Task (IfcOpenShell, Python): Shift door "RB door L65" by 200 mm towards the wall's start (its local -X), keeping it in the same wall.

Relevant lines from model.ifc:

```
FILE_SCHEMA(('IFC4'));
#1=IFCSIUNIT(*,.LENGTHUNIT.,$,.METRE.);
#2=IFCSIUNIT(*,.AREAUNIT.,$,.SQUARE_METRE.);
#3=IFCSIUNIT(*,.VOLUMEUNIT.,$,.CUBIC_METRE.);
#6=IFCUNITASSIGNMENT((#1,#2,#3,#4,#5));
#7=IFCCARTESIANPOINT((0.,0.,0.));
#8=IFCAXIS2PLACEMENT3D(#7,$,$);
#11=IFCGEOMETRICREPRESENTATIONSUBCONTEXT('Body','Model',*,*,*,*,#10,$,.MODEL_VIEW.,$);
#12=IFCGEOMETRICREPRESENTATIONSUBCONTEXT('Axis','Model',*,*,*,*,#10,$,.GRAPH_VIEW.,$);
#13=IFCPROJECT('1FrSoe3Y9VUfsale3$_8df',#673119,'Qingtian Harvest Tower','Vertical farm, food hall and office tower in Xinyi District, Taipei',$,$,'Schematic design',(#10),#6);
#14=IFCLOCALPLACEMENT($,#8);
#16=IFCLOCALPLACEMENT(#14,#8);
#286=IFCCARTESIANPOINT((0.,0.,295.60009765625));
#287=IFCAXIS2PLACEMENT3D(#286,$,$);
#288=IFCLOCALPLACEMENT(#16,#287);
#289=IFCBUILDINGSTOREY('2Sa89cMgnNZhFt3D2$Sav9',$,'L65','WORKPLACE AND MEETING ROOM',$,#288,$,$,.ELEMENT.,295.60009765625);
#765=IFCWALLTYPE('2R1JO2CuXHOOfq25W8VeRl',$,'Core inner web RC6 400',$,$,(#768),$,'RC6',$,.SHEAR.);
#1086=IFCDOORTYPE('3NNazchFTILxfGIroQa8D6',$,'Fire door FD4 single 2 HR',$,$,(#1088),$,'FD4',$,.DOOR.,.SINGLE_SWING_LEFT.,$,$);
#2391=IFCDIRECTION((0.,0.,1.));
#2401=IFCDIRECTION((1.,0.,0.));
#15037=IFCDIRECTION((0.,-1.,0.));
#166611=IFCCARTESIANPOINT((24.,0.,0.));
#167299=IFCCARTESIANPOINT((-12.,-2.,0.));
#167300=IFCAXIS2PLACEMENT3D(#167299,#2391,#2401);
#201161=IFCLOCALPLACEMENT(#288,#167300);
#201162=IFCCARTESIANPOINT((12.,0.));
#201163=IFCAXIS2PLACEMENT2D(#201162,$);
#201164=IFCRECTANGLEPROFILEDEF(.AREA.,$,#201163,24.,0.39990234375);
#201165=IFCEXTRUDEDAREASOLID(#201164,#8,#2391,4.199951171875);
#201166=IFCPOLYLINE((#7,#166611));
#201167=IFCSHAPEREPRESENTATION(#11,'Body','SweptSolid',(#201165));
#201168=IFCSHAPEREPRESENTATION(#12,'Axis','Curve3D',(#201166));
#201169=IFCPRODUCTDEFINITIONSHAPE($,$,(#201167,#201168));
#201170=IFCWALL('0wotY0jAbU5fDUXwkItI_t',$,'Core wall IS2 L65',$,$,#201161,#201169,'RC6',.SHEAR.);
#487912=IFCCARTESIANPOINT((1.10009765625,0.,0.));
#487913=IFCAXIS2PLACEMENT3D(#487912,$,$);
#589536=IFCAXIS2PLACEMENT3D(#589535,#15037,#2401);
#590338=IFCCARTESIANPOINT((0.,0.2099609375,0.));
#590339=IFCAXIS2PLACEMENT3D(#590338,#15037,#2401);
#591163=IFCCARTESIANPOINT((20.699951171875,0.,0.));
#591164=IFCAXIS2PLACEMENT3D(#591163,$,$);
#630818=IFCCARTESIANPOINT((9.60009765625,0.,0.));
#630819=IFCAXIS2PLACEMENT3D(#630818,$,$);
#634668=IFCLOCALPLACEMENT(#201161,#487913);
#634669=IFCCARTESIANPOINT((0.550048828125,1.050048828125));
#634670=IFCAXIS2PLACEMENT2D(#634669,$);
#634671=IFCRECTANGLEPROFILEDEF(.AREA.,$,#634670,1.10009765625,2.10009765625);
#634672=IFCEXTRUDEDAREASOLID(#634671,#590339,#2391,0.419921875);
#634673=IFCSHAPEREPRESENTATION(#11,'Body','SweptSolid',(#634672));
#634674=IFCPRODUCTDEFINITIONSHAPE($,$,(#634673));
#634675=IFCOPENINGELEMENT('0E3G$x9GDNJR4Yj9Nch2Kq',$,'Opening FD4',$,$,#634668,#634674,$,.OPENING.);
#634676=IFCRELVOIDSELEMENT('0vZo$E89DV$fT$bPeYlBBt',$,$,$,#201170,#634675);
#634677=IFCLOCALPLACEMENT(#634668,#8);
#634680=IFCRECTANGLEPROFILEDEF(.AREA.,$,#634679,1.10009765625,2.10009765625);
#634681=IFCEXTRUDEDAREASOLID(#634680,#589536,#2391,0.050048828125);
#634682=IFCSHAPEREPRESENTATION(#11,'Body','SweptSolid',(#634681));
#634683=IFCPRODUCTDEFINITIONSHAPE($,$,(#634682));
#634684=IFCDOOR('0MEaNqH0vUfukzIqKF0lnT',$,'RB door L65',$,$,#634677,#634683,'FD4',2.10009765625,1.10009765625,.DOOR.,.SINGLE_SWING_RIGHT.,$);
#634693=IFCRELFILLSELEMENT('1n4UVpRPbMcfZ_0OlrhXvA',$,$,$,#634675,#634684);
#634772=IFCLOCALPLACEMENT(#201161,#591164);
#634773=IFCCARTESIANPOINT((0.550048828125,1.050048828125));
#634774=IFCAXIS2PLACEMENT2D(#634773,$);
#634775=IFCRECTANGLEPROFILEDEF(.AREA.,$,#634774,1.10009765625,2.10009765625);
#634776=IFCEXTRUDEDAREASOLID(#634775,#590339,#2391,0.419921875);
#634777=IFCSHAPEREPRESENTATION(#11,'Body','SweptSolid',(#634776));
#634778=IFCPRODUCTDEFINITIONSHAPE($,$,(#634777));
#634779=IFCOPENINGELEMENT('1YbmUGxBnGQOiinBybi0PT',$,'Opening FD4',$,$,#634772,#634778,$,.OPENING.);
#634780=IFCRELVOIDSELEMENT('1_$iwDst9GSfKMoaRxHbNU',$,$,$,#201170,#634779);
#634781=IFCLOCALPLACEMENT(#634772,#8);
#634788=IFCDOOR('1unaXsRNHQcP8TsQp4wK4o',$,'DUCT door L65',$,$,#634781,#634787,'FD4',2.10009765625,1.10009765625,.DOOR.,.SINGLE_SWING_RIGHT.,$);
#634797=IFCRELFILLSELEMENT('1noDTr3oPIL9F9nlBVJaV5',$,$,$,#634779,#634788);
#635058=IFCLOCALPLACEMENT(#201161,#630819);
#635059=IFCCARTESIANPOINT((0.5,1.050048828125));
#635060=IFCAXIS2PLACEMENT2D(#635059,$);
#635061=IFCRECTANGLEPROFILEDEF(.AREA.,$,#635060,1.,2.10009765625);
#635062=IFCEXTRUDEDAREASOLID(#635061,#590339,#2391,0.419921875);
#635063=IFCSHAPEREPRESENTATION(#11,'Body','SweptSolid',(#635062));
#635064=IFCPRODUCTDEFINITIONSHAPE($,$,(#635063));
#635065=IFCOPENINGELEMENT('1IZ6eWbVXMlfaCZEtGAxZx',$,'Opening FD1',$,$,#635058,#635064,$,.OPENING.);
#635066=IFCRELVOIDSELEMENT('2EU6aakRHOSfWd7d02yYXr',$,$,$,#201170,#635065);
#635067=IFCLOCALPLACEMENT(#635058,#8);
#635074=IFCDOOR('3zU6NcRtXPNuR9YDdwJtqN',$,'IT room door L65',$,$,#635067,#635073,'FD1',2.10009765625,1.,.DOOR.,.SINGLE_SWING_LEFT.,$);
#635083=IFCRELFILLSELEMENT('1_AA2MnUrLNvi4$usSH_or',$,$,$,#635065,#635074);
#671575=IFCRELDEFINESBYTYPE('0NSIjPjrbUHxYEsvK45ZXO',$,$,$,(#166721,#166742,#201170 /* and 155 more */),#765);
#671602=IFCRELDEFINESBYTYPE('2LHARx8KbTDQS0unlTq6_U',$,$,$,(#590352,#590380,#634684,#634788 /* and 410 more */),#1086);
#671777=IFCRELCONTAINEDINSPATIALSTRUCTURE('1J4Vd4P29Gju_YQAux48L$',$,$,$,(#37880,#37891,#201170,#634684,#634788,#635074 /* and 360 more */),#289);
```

```python
import ifcopenshell
import ifcopenshell.api.geometry
import ifcopenshell.util.placement

model = ifcopenshell.open("model.ifc")

door = model.by_guid("0MEaNqH0vUfukzIqKF0lnT")
opening = door.FillsVoids[0].RelatingOpeningElement
wall = opening.VoidsElements[0].RelatingBuildingElement

wall_matrix = ifcopenshell.util.placement.get_local_placement(wall.ObjectPlacement)
shift = wall_matrix[:3, 0] * -0.2
before = ifcopenshell.util.placement.get_local_placement(door.ObjectPlacement)[:3, 3].copy()

# The door is placed relative to its opening, so it follows when the opening moves.
matrix = ifcopenshell.util.placement.get_local_placement(opening.ObjectPlacement)
matrix[:3, 3] += shift
ifcopenshell.api.geometry.edit_object_placement(
    model, product=opening, matrix=matrix, is_si=False, should_transform_children=True
)

after = ifcopenshell.util.placement.get_local_placement(door.ObjectPlacement)[:3, 3]
print("door moved by", (after - before).round(3) + 0.0)

model.write("model-out.ifc")
```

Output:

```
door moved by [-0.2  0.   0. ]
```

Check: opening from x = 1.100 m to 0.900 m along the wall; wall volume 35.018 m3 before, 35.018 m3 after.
